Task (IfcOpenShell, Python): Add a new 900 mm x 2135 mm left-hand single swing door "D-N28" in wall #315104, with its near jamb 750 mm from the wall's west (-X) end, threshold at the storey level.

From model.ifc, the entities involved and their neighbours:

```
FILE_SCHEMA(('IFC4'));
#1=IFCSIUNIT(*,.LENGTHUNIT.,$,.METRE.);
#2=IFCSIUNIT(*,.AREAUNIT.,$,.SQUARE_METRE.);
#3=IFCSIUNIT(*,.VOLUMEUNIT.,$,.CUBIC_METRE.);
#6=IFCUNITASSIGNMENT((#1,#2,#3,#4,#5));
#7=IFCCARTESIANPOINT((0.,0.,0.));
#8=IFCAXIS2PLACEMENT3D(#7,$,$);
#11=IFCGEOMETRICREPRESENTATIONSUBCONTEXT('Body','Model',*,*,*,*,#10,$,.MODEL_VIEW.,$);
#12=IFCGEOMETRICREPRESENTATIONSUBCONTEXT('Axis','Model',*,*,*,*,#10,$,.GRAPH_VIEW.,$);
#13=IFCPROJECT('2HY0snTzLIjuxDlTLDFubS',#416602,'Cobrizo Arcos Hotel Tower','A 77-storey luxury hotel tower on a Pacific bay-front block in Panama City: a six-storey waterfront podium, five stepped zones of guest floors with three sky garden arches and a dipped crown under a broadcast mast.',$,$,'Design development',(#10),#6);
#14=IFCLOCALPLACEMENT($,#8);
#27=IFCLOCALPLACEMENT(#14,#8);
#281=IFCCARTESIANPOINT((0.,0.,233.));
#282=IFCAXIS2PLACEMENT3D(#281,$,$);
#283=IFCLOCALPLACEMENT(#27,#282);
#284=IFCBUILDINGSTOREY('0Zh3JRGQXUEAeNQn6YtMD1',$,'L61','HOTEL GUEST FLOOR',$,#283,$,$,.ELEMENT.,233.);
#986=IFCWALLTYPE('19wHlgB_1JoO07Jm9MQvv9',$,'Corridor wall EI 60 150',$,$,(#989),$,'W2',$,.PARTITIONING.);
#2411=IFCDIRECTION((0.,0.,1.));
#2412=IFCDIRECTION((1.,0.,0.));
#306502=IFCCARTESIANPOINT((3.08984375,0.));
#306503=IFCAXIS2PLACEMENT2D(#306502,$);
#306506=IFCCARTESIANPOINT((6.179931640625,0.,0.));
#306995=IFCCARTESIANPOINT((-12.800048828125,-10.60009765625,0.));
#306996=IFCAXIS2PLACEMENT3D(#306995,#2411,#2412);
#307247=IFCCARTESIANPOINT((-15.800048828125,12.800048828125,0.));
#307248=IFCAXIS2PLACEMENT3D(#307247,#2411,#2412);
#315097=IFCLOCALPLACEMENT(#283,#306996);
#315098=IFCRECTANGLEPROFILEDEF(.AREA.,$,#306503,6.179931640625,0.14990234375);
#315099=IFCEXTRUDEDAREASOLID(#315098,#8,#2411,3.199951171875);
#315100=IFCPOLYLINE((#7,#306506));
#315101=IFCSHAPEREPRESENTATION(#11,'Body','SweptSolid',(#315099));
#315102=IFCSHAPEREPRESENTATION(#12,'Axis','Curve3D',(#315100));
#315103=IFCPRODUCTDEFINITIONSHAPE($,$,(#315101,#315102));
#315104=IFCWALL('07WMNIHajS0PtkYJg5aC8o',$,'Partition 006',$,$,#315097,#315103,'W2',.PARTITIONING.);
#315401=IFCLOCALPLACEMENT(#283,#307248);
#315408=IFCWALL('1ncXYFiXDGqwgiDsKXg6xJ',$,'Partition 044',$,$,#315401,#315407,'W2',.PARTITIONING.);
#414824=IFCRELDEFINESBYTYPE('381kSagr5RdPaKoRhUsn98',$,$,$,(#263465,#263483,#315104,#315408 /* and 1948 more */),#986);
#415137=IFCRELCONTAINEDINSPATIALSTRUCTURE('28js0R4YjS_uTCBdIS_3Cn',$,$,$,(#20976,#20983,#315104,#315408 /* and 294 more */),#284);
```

```python
import numpy as np
import ifcopenshell
import ifcopenshell.api.feature
import ifcopenshell.api.geometry
import ifcopenshell.api.root
import ifcopenshell.api.spatial
import ifcopenshell.geom
import ifcopenshell.util.element
import ifcopenshell.util.placement
import ifcopenshell.util.representation
import ifcopenshell.util.shape
import ifcopenshell.util.unit

model = ifcopenshell.open("model.ifc")
unit_scale = ifcopenshell.util.unit.calculate_unit_scale(model)
settings = ifcopenshell.geom.settings()


def volume(element):
    """Net volume in cubic metres, openings subtracted."""
    shape = ifcopenshell.geom.create_shape(settings, element)
    return ifcopenshell.util.shape.get_volume(shape.geometry)


wall = model.by_guid("07WMNIHajS0PtkYJg5aC8o")
storey = ifcopenshell.util.element.get_container(wall, ifc_class="IfcBuildingStorey")
context = ifcopenshell.util.representation.get_context(model, "Model", "Body", "MODEL_VIEW")
before = volume(wall)

width, height, from_end, sill = 0.9, 2.135, 0.75, 0.0  # metres

# The wall runs along its own X axis, and the end named is its -X end.
wall_shape = ifcopenshell.geom.create_shape(settings, wall)
x, y, z = ifcopenshell.util.shape.get_vertices(wall_shape.geometry).T
start = x.min() + from_end
face, thickness = float(y.min()), float(y.max() - y.min())
wall_matrix = ifcopenshell.util.placement.get_local_placement(wall.ObjectPlacement)
level = ifcopenshell.util.placement.get_local_placement(storey.ObjectPlacement)[2, 3]


def in_wall(x, y):
    """Placement at x, y metres in the wall's axes, at sill height."""
    matrix = wall_matrix.copy()
    matrix[:, 3] = wall_matrix @ np.array([x / unit_scale, y / unit_scale, 0.0, 1.0])
    matrix[2, 3] = level + sill / unit_scale
    return matrix


# Opening: a box that overshoots both wall faces by 50 mm.
opening = ifcopenshell.api.root.create_entity(model, ifc_class="IfcOpeningElement", predefined_type="OPENING")
box = ifcopenshell.api.geometry.add_wall_representation(
    model, context=context, length=width, height=height, thickness=thickness + 0.1
)
ifcopenshell.api.geometry.assign_representation(model, product=opening, representation=box)
ifcopenshell.api.geometry.edit_object_placement(model, product=opening, matrix=in_wall(start, face - 0.05), is_si=False)
ifcopenshell.api.feature.add_feature(model, feature=opening, element=wall)

door = ifcopenshell.api.root.create_entity(model, ifc_class="IfcDoor", name="D-N28", predefined_type="DOOR")
door.OverallWidth, door.OverallHeight = width / unit_scale, height / unit_scale
door.OperationType = "SINGLE_SWING_LEFT"
body = ifcopenshell.api.geometry.add_door_representation(
    model,
    context=context,
    overall_width=door.OverallWidth,
    overall_height=door.OverallHeight,
    operation_type="SINGLE_SWING_LEFT",
    lining_properties={"LiningDepth": thickness / unit_scale, "ThresholdDepth": thickness / unit_scale},
)
ifcopenshell.api.geometry.assign_representation(model, product=door, representation=body)
ifcopenshell.api.spatial.assign_container(model, products=[door], relating_structure=storey)
ifcopenshell.api.feature.add_filling(model, opening=opening, element=door)

# The lining spans the wall, so the door starts at the wall face.
ifcopenshell.api.geometry.edit_object_placement(model, product=door, matrix=in_wall(start, face), is_si=False)

after = volume(wall)

print(f"wall volume {before:.3f} -> {after:.3f} m3")

model.write("model_v2.ifc")
```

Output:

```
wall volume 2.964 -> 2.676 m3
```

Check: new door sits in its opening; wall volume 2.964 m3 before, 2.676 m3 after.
